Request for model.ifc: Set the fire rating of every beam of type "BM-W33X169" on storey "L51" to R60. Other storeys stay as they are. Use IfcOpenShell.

First a look at what the model holds.

```python
import ifcopenshell
import ifcopenshell.util.element

model = ifcopenshell.open("model.ifc")
print(model.schema)
storey = next(s for s in model.by_type("IfcBuildingStorey") if s.Name == "L51")
beams = [e for e in ifcopenshell.util.element.get_decomposition(storey) if e.is_a("IfcBeam")]
seen = {}
for e in beams:
    element_type = ifcopenshell.util.element.get_type(e)
    key = (element_type.Name if element_type != e and element_type else None, ifcopenshell.util.element.get_pset(e, "Pset_BeamCommon", "FireRating"))
    seen[key] = seen.get(key, 0) + 1
for (name, value), count in sorted(seen.items(), key=str):
    print(count, "x", name, "|", value)
```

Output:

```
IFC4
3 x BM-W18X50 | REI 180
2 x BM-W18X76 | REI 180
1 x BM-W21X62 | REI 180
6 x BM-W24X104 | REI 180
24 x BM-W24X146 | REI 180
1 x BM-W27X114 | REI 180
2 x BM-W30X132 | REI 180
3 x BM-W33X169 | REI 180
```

```python
import ifcopenshell
import ifcopenshell.api.pset
import ifcopenshell.util.element

model = ifcopenshell.open("model.ifc")

storey = next(s for s in model.by_type("IfcBuildingStorey") if s.Name == "L51")
beams = [e for e in ifcopenshell.util.element.get_decomposition(storey) if e.is_a("IfcBeam")]

count = 0
for e in beams:
    element_type = ifcopenshell.util.element.get_type(e)
    if element_type in (None, e) or element_type.Name != "BM-W33X169":
        continue
    found = ifcopenshell.util.element.get_pset(e, "Pset_BeamCommon", should_inherit=False)
    if found:
        pset = model.by_id(found["id"])
        if len(ifcopenshell.util.element.get_elements_by_pset(pset)) > 1:
            pset = ifcopenshell.api.pset.unshare_pset(model, products=[e], pset=pset)[0]
    else:
        pset = ifcopenshell.api.pset.add_pset(model, product=e, name="Pset_BeamCommon")
    ifcopenshell.api.pset.edit_pset(model, pset=pset, properties={"FireRating": "R60"})
    count += 1

print(count, "beams updated")

model.write("model_edited.ifc")
```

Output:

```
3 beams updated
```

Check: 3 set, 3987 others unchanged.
